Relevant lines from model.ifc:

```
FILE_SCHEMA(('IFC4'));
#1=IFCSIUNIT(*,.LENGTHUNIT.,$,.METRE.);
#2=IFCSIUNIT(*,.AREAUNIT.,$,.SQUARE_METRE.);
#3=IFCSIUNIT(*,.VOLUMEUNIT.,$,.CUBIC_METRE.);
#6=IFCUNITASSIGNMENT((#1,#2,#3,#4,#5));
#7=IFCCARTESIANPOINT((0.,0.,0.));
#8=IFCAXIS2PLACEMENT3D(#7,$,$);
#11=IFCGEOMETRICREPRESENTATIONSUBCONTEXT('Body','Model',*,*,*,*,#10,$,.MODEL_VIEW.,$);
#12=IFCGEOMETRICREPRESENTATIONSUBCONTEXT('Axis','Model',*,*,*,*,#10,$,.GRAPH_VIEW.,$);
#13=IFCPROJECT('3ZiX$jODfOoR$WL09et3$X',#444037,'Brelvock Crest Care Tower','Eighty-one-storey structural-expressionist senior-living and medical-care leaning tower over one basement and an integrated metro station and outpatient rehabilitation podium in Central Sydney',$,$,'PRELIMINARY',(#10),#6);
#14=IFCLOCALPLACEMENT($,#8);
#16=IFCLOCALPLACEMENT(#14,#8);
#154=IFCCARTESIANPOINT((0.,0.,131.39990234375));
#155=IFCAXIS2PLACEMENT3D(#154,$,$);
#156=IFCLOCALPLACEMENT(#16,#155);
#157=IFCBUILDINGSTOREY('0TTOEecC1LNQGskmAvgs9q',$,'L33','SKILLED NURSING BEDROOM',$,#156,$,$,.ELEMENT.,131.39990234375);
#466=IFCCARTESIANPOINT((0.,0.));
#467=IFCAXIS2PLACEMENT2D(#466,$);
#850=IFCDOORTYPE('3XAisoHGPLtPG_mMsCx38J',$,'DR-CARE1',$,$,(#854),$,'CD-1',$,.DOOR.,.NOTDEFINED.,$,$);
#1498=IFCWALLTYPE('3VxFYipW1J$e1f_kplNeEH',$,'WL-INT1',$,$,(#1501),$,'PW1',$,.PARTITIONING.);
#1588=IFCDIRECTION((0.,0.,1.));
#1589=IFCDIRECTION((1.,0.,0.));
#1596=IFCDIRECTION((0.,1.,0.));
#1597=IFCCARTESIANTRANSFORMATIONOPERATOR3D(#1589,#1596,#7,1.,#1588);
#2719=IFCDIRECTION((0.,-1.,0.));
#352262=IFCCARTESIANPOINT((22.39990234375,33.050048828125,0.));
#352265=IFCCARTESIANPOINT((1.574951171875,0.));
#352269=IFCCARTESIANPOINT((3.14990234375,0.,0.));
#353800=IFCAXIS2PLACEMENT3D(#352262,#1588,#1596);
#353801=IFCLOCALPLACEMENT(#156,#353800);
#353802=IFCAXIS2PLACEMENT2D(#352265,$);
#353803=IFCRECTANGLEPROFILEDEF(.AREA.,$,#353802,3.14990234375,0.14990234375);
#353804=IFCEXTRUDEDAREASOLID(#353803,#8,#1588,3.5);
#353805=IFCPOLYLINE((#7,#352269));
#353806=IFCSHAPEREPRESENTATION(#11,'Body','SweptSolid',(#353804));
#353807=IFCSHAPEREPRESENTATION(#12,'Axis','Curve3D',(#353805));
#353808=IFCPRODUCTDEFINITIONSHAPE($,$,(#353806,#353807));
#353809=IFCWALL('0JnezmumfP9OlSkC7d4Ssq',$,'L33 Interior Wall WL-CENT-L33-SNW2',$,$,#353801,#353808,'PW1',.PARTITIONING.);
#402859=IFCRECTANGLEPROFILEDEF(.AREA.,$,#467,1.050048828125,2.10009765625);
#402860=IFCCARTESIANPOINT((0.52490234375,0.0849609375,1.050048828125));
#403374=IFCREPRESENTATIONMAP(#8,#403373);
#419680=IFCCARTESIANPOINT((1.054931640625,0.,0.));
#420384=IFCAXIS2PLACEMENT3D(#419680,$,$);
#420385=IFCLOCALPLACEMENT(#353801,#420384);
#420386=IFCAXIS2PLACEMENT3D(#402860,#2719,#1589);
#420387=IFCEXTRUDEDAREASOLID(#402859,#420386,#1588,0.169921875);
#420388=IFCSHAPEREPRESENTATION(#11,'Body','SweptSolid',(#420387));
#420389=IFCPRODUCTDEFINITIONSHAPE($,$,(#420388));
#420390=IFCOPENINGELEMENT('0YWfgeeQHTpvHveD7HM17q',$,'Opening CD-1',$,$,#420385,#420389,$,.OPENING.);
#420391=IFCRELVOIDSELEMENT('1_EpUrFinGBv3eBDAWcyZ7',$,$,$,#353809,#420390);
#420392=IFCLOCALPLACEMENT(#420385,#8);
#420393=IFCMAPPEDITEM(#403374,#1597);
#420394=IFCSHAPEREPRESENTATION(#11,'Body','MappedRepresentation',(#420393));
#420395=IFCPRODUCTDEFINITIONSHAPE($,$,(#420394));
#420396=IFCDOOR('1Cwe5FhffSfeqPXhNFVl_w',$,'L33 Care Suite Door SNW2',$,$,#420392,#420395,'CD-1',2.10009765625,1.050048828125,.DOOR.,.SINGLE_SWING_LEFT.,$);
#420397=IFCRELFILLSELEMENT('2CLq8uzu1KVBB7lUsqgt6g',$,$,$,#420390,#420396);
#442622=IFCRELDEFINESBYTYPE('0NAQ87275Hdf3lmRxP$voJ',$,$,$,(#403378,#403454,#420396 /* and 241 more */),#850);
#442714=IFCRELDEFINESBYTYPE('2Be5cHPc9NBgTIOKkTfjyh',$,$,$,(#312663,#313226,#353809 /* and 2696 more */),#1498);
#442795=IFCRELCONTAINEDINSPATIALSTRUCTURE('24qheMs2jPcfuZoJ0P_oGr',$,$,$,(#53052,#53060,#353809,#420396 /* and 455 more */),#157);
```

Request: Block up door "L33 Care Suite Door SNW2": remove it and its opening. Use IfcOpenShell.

```python
import ifcopenshell
import ifcopenshell.api.feature
import ifcopenshell.api.root
import ifcopenshell.geom
import ifcopenshell.util.shape

model = ifcopenshell.open("model.ifc")
settings = ifcopenshell.geom.settings()


def volume(element):
    """Net volume in cubic metres, openings subtracted."""
    shape = ifcopenshell.geom.create_shape(settings, element)
    return ifcopenshell.util.shape.get_volume(shape.geometry)


door = model.by_guid("1Cwe5FhffSfeqPXhNFVl_w")
opening = door.FillsVoids[0].RelatingOpeningElement
wall = opening.VoidsElements[0].RelatingBuildingElement
before = volume(wall)

ifcopenshell.api.root.remove_product(model, product=door)
ifcopenshell.api.feature.remove_feature(model, feature=opening)

after = volume(wall)

print(f"wall volume {before:.3f} -> {after:.3f} m3")

model.write("model_v2.ifc")
```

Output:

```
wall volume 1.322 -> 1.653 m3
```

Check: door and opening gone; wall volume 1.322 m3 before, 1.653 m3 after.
